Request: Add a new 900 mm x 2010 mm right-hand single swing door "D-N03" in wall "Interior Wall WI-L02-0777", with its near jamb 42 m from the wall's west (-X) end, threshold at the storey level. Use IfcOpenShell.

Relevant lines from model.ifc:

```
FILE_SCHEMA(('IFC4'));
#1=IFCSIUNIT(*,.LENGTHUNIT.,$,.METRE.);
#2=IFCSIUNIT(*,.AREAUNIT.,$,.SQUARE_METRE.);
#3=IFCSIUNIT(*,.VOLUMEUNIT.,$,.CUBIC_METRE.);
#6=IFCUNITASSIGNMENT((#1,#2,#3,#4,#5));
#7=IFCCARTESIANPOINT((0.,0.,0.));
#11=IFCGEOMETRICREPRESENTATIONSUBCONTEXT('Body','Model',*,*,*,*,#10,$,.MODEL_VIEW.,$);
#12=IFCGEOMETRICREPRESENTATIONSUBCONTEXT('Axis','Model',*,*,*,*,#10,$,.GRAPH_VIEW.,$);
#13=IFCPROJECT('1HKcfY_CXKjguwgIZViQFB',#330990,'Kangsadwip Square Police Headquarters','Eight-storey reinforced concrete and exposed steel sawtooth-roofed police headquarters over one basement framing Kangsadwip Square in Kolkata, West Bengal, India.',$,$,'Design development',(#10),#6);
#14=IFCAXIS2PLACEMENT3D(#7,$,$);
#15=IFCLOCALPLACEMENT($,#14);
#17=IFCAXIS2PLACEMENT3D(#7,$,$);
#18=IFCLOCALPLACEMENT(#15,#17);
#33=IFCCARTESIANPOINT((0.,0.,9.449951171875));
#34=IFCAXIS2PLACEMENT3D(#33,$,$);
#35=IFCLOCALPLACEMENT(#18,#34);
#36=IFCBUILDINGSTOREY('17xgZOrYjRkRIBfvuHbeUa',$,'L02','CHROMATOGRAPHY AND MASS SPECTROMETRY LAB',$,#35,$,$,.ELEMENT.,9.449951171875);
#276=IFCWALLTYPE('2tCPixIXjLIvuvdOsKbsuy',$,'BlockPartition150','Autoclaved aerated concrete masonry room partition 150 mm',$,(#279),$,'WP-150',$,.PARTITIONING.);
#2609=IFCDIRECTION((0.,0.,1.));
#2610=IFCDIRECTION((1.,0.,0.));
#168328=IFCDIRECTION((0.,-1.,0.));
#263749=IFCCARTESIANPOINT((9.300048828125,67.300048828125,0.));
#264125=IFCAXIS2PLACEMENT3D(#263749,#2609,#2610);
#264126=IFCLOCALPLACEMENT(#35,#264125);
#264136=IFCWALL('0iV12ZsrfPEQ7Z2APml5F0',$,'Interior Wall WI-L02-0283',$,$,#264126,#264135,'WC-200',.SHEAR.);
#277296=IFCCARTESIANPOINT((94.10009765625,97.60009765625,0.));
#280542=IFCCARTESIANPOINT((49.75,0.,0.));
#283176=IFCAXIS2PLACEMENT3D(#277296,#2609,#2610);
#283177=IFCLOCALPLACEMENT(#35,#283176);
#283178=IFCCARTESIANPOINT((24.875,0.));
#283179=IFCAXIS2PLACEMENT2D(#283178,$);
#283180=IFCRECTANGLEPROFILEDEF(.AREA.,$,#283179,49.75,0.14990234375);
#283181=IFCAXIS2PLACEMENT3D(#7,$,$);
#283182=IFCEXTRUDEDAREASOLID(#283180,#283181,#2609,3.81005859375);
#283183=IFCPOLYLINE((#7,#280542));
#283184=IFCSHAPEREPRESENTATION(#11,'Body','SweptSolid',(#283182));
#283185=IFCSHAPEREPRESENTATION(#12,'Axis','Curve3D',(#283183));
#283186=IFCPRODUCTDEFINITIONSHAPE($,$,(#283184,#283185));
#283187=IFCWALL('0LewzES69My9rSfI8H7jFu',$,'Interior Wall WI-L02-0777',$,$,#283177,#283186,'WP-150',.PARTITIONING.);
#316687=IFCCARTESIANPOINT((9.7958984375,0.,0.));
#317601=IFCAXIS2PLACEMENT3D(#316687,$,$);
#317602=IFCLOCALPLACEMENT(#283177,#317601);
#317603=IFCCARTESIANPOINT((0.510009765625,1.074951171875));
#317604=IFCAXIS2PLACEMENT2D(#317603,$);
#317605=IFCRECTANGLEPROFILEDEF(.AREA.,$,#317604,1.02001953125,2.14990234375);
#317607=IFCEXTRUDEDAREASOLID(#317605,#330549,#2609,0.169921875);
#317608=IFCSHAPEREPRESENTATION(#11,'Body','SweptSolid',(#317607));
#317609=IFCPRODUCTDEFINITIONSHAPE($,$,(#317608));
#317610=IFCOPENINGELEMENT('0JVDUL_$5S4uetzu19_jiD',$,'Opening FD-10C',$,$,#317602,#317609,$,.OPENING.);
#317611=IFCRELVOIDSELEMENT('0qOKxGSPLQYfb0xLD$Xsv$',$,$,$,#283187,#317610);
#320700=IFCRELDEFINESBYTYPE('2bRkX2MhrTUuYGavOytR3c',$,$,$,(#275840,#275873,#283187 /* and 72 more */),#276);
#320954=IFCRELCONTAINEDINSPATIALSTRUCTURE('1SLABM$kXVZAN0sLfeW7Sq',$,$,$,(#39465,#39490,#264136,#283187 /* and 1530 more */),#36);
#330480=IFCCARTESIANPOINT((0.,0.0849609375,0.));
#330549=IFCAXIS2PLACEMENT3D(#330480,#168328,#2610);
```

```python
import numpy as np
import ifcopenshell
import ifcopenshell.api.feature
import ifcopenshell.api.geometry
import ifcopenshell.api.root
import ifcopenshell.api.spatial
import ifcopenshell.geom
import ifcopenshell.util.element
import ifcopenshell.util.placement
import ifcopenshell.util.representation
import ifcopenshell.util.shape
import ifcopenshell.util.unit

model = ifcopenshell.open("model.ifc")
unit_scale = ifcopenshell.util.unit.calculate_unit_scale(model)
settings = ifcopenshell.geom.settings()


def volume(element):
    """Net volume in cubic metres, openings subtracted."""
    shape = ifcopenshell.geom.create_shape(settings, element)
    return ifcopenshell.util.shape.get_volume(shape.geometry)


wall = model.by_id(283187)
storey = ifcopenshell.util.element.get_container(wall, ifc_class="IfcBuildingStorey")
context = ifcopenshell.util.representation.get_context(model, "Model", "Body", "MODEL_VIEW")
before = volume(wall)

width, height, from_end, sill = 0.9, 2.01, 42, 0.0  # metres

# The wall runs along its own X axis, and the end named is its -X end.
wall_shape = ifcopenshell.geom.create_shape(settings, wall)
x, y, z = ifcopenshell.util.shape.get_vertices(wall_shape.geometry).T
start = x.min() + from_end
face, thickness = float(y.min()), float(y.max() - y.min())
wall_matrix = ifcopenshell.util.placement.get_local_placement(wall.ObjectPlacement)
level = ifcopenshell.util.placement.get_local_placement(storey.ObjectPlacement)[2, 3]


def in_wall(x, y):
    """Placement at x, y metres in the wall's axes, at sill height."""
    matrix = wall_matrix.copy()
    matrix[:, 3] = wall_matrix @ np.array([x / unit_scale, y / unit_scale, 0.0, 1.0])
    matrix[2, 3] = level + sill / unit_scale
    return matrix


# Opening: a box that overshoots both wall faces by 50 mm.
opening = ifcopenshell.api.root.create_entity(model, ifc_class="IfcOpeningElement", predefined_type="OPENING")
box = ifcopenshell.api.geometry.add_wall_representation(
    model, context=context, length=width, height=height, thickness=thickness + 0.1
)
ifcopenshell.api.geometry.assign_representation(model, product=opening, representation=box)
ifcopenshell.api.geometry.edit_object_placement(model, product=opening, matrix=in_wall(start, face - 0.05), is_si=False)
ifcopenshell.api.feature.add_feature(model, feature=opening, element=wall)

door = ifcopenshell.api.root.create_entity(model, ifc_class="IfcDoor", name="D-N03", predefined_type="DOOR")
door.OverallWidth, door.OverallHeight = width / unit_scale, height / unit_scale
door.OperationType = "SINGLE_SWING_RIGHT"
body = ifcopenshell.api.geometry.add_door_representation(
    model,
    context=context,
    overall_width=door.OverallWidth,
    overall_height=door.OverallHeight,
    operation_type="SINGLE_SWING_RIGHT",
    lining_properties={"LiningDepth": thickness / unit_scale, "ThresholdDepth": thickness / unit_scale},
)
ifcopenshell.api.geometry.assign_representation(model, product=door, representation=body)
ifcopenshell.api.spatial.assign_container(model, products=[door], relating_structure=storey)
ifcopenshell.api.feature.add_filling(model, opening=opening, element=door)

# The lining spans the wall, so the door starts at the wall face.
ifcopenshell.api.geometry.edit_object_placement(model, product=door, matrix=in_wall(start, face), is_si=False)

after = volume(wall)

print(f"wall volume {before:.3f} -> {after:.3f} m3")

model.write("model_v2.ifc")
```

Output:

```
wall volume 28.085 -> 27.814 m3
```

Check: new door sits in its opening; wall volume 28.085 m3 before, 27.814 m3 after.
